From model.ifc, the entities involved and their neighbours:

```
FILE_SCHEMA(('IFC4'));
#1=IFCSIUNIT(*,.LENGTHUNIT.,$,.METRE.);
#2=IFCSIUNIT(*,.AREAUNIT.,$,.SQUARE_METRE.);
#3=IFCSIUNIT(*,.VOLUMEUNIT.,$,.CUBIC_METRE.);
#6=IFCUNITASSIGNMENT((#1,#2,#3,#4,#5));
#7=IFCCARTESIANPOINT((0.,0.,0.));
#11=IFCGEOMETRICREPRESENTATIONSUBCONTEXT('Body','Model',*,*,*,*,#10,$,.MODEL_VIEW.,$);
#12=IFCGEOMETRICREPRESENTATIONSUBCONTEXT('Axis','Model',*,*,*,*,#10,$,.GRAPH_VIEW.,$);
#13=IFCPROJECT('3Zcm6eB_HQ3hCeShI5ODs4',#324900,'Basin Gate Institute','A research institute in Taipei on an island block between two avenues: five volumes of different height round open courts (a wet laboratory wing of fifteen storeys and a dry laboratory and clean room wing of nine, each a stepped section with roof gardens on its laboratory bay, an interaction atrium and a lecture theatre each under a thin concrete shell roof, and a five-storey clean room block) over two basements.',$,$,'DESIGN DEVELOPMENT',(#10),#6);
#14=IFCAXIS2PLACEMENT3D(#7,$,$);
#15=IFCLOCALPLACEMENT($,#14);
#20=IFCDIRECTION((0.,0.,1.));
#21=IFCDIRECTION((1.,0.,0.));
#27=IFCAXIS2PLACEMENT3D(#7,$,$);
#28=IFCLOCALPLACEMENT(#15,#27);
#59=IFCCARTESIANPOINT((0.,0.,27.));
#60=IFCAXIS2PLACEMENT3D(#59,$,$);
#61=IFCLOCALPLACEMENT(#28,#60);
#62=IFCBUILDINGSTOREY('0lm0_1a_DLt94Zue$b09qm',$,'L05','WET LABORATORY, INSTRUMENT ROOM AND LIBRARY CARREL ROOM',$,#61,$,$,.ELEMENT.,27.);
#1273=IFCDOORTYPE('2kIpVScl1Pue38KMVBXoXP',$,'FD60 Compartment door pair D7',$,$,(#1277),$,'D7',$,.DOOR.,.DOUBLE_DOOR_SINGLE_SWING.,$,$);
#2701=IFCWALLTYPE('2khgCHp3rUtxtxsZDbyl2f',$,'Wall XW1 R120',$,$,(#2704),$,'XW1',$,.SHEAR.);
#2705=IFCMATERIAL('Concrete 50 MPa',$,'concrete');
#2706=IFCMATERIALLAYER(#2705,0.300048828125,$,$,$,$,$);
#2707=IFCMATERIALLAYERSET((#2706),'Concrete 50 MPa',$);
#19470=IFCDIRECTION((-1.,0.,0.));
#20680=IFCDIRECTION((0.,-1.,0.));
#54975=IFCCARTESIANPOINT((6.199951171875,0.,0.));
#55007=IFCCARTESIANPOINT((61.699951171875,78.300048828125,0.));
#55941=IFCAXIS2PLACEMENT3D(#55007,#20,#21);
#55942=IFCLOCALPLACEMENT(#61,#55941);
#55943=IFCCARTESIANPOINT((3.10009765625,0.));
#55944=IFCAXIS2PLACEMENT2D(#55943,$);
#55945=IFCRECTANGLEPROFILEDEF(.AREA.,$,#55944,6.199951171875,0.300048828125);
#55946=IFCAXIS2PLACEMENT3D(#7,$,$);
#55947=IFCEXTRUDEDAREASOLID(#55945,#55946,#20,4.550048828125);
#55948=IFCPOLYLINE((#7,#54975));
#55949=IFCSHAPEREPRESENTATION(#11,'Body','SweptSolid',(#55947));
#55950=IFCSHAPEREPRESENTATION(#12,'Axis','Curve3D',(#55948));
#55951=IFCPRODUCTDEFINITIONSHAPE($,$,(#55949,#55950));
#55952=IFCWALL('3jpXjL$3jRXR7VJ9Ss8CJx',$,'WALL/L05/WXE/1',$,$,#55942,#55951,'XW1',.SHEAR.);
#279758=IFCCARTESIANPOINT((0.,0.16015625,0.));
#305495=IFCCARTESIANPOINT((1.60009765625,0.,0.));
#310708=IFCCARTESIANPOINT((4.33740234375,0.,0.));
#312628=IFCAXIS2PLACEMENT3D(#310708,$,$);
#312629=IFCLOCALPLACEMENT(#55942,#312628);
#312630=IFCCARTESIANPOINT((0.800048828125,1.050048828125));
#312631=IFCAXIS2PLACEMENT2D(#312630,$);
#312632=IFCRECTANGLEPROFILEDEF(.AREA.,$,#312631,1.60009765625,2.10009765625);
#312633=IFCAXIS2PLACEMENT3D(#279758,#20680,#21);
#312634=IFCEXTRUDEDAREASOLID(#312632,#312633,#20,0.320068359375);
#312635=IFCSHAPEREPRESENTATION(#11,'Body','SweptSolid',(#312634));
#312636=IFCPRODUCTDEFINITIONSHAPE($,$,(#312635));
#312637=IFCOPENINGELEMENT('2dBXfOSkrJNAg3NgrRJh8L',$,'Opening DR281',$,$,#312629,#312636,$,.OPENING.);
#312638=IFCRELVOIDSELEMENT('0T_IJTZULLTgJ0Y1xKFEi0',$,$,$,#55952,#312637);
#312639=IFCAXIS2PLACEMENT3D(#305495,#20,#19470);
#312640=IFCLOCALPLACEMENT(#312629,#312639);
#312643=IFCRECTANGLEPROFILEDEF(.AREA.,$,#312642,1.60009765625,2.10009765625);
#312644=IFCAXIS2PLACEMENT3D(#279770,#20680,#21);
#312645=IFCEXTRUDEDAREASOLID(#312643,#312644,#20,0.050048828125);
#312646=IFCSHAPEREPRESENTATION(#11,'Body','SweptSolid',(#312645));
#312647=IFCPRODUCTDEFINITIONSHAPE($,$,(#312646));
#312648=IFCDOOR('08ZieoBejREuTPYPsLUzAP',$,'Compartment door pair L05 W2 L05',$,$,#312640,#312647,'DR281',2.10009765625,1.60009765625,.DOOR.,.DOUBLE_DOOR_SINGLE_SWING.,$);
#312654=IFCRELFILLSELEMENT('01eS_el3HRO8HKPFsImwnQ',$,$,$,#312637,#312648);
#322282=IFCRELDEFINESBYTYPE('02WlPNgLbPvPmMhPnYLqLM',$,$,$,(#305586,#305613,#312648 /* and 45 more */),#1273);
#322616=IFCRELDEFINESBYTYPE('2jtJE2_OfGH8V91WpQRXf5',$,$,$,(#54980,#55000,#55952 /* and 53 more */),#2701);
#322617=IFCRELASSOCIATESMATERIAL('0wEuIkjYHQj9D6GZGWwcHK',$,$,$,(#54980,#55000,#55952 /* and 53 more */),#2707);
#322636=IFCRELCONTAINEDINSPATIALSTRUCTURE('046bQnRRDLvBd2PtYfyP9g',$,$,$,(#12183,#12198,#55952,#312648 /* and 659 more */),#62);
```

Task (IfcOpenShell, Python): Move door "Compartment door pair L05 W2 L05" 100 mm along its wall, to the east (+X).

```python
import ifcopenshell
import ifcopenshell.api.geometry
import ifcopenshell.util.placement
import ifcopenshell.util.unit

model = ifcopenshell.open("model.ifc")
unit_scale = ifcopenshell.util.unit.calculate_unit_scale(model)

door = model.by_id(312648)
opening = door.FillsVoids[0].RelatingOpeningElement
wall = opening.VoidsElements[0].RelatingBuildingElement

wall_matrix = ifcopenshell.util.placement.get_local_placement(wall.ObjectPlacement)
shift = wall_matrix[:3, 0] * 0.1 / unit_scale
before = ifcopenshell.util.placement.get_local_placement(door.ObjectPlacement)[:3, 3].copy()

# The door is placed relative to its opening, so it follows when the opening moves.
matrix = ifcopenshell.util.placement.get_local_placement(opening.ObjectPlacement)
matrix[:3, 3] += shift
ifcopenshell.api.geometry.edit_object_placement(
    model, product=opening, matrix=matrix, is_si=False, should_transform_children=True
)

after = ifcopenshell.util.placement.get_local_placement(door.ObjectPlacement)[:3, 3]
print("door moved by", (after - before).round(3) + 0.0)

model.write("model_updated.ifc")
```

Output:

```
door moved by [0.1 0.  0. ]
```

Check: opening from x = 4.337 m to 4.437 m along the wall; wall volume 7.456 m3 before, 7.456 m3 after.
